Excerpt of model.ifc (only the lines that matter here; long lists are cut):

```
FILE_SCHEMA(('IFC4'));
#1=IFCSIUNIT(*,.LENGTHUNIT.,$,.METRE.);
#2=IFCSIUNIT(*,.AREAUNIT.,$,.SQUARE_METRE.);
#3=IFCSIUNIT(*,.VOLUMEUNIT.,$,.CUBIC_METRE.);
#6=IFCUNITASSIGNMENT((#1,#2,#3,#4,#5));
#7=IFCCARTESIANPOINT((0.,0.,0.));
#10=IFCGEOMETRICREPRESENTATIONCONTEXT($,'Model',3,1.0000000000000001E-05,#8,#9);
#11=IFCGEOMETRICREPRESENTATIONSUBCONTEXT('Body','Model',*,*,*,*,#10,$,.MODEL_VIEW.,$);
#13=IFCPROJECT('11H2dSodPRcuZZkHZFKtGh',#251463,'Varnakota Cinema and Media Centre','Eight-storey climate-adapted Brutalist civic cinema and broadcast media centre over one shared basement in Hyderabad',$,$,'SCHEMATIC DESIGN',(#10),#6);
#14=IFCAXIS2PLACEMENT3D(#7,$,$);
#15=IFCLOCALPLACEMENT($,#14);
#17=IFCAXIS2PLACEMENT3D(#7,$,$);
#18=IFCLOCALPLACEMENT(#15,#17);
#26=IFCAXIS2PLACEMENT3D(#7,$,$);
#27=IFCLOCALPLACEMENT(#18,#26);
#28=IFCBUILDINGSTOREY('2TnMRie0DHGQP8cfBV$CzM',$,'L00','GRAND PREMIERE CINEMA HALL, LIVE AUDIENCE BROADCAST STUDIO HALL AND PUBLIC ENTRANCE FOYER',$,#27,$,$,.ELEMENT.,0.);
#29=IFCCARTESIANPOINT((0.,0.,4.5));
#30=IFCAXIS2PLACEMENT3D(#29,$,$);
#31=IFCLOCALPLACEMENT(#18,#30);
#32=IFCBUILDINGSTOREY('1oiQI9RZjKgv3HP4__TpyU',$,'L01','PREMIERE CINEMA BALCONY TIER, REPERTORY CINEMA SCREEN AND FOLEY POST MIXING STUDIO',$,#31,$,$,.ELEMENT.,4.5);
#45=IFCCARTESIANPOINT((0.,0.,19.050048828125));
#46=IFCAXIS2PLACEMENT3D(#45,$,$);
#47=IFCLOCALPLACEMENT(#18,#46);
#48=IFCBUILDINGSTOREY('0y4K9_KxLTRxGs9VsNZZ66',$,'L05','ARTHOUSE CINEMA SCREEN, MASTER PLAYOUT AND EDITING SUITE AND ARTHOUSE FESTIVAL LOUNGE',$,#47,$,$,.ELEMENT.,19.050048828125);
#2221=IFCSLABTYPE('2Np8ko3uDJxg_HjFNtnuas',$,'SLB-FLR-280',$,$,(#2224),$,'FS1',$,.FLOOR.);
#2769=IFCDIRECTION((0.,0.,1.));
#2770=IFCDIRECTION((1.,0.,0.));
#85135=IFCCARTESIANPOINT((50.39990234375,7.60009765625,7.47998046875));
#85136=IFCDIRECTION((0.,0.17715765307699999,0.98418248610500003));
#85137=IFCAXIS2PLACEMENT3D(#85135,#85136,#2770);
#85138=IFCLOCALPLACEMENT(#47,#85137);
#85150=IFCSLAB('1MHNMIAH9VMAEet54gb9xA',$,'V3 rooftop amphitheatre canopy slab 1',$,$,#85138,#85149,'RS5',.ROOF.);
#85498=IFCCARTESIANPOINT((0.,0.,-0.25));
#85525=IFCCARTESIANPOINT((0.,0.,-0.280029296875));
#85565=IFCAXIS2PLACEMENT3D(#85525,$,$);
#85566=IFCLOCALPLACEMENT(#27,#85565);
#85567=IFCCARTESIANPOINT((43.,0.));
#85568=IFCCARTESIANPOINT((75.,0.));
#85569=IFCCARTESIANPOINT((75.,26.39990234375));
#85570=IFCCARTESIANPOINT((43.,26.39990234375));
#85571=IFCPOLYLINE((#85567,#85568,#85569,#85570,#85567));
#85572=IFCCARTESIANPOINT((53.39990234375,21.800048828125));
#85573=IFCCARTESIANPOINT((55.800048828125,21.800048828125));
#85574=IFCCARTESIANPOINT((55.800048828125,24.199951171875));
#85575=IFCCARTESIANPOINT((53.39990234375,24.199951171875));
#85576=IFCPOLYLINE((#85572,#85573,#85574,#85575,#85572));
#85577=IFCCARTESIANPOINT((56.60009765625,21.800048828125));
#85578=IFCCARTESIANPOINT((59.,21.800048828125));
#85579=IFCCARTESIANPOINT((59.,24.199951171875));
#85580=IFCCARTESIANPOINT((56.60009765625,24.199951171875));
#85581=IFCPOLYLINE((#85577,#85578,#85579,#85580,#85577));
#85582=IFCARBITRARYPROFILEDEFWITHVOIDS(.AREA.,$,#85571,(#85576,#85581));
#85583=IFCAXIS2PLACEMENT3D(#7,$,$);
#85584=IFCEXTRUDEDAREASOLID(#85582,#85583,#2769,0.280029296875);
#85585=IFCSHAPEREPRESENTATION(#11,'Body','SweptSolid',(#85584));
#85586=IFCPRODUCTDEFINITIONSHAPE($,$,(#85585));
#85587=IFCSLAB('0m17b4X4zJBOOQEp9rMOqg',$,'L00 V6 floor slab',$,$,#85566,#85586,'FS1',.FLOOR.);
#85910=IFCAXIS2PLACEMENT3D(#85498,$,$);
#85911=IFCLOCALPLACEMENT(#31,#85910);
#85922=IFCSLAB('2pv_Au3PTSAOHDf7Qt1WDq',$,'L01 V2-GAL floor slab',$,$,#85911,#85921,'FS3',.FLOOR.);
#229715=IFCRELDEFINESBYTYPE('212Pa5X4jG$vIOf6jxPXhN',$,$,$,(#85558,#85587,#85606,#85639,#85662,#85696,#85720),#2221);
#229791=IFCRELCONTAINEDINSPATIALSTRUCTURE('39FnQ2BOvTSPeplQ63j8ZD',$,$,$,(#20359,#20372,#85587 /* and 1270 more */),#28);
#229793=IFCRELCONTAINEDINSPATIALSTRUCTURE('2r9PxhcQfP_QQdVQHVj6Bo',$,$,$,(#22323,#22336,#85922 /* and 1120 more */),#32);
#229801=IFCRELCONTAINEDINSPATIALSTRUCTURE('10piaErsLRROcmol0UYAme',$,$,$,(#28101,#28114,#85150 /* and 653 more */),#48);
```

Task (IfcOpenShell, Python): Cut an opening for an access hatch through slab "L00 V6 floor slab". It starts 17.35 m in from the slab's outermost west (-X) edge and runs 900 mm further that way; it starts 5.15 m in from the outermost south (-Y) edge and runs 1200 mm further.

```python
import numpy as np
import ifcopenshell
import ifcopenshell.api.feature
import ifcopenshell.api.geometry
import ifcopenshell.api.root
import ifcopenshell.geom
import ifcopenshell.util.placement
import ifcopenshell.util.representation
import ifcopenshell.util.shape
import ifcopenshell.util.unit

model = ifcopenshell.open("model.ifc")
unit_scale = ifcopenshell.util.unit.calculate_unit_scale(model)
settings = ifcopenshell.geom.settings()


def volume(element):
    """Net volume in cubic metres, openings subtracted."""
    shape = ifcopenshell.geom.create_shape(settings, element)
    return ifcopenshell.util.shape.get_volume(shape.geometry)


slab = model.by_guid("0m17b4X4zJBOOQEp9rMOqg")
before = volume(slab)

# Extent in the slab's own axes, in metres. The edges named are its -X and -Y sides.
slab_shape = ifcopenshell.geom.create_shape(settings, slab)
vertices = ifcopenshell.util.shape.get_vertices(slab_shape.geometry)
x_min, y_min, bottom = vertices.min(axis=0)
top = vertices[:, 2].max()

opening = ifcopenshell.api.root.create_entity(model, ifc_class="IfcOpeningElement", name="Access hatch opening", predefined_type="OPENING")
context = ifcopenshell.util.representation.get_context(model, "Model", "Body", "MODEL_VIEW")
width, depth = 0.9, 1.2
outline = [(0.0, 0.0), (width, 0.0), (width, depth), (0.0, depth), (0.0, 0.0)]
# Overshoot both faces by 50 mm so the cut is clean.
shape = ifcopenshell.api.geometry.add_slab_representation(
    model, context=context, depth=top - bottom + 0.1, polyline=outline
)
ifcopenshell.api.geometry.assign_representation(model, product=opening, representation=shape)

matrix = ifcopenshell.util.placement.get_local_placement(slab.ObjectPlacement)
matrix[:, 3] = matrix @ np.append(np.array([x_min + 17.35, y_min + 5.15, bottom - 0.05]) / unit_scale, 1.0)
ifcopenshell.api.geometry.edit_object_placement(model, product=opening, matrix=matrix, is_si=False)
ifcopenshell.api.feature.add_feature(model, feature=opening, element=slab)

after = volume(slab)

print(f"slab volume {before:.3f} -> {after:.3f} m3")

model.write("model_v2.ifc")
```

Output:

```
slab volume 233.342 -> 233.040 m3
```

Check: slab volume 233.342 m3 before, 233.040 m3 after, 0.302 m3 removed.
